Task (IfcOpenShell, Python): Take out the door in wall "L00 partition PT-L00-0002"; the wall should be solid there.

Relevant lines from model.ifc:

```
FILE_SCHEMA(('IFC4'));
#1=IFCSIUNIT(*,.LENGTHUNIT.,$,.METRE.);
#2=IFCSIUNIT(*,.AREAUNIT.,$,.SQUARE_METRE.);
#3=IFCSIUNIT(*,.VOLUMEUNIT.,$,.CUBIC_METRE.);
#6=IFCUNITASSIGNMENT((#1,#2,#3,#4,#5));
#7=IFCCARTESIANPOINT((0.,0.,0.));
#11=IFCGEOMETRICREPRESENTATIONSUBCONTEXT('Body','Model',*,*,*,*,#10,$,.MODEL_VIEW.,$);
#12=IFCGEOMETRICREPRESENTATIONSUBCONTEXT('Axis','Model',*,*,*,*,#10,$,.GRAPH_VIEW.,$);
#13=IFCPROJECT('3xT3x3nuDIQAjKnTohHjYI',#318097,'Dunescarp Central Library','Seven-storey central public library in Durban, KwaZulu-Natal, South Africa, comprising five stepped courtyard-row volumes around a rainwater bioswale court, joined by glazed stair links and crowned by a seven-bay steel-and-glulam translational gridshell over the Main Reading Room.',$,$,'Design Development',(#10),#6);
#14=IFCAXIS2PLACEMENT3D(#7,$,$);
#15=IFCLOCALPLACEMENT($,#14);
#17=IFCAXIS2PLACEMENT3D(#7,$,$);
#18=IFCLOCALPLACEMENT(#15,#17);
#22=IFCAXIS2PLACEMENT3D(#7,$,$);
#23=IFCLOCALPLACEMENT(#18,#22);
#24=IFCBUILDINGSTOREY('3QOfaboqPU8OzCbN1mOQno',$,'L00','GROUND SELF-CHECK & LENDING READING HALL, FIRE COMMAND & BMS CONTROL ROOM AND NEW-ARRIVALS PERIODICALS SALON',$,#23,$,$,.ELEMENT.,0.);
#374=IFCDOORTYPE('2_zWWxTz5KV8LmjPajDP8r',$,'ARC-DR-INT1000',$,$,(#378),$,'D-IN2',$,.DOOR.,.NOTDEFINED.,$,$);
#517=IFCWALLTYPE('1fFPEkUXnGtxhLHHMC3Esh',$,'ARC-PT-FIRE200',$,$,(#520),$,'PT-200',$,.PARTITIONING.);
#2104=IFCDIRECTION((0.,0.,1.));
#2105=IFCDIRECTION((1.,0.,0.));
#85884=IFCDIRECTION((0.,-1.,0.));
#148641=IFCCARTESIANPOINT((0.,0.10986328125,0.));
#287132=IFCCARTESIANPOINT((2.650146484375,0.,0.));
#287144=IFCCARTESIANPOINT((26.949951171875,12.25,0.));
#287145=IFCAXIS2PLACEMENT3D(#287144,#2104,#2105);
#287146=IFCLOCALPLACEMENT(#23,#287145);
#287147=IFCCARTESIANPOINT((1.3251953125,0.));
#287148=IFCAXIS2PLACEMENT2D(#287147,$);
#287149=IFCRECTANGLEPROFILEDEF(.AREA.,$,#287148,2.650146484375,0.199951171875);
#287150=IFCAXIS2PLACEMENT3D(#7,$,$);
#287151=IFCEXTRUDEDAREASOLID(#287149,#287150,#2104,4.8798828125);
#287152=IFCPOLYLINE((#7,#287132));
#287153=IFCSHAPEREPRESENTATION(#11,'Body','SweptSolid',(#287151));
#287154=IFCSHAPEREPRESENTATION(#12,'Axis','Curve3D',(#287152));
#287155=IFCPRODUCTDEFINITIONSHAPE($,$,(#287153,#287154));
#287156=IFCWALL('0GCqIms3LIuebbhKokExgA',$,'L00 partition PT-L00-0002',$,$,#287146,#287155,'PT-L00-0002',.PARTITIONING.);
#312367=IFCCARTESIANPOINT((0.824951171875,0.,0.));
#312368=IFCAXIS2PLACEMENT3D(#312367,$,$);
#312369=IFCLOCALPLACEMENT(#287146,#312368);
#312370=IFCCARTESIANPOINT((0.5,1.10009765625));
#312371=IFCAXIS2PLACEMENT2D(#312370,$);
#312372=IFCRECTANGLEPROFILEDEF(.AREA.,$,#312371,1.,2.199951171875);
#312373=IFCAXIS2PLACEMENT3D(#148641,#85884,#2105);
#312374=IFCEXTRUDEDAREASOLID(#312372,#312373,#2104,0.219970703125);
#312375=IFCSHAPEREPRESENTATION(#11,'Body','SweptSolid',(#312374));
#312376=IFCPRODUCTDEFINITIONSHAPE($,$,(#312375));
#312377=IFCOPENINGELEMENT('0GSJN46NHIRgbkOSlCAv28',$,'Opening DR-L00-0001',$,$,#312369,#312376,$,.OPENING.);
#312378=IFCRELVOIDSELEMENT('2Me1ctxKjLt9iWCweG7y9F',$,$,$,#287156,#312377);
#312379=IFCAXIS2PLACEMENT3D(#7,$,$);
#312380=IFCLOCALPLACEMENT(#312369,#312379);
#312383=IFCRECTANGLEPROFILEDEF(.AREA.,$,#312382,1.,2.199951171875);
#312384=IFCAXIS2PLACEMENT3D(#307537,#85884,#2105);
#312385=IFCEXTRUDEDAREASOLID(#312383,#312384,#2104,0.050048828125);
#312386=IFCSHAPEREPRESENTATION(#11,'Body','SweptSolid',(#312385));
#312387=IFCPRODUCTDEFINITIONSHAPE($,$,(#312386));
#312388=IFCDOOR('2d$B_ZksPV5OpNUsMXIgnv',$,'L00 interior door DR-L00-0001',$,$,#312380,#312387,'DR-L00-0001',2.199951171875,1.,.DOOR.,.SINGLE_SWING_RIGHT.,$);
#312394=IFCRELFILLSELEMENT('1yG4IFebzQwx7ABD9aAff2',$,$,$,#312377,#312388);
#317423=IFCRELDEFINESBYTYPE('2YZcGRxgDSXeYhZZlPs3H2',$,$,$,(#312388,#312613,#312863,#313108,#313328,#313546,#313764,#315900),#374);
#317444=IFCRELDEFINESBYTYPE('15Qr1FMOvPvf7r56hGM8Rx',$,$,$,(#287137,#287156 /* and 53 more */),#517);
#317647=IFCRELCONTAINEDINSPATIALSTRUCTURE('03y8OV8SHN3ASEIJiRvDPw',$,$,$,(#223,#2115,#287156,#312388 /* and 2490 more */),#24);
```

```python
import ifcopenshell
import ifcopenshell.api.feature
import ifcopenshell.api.root
import ifcopenshell.geom
import ifcopenshell.util.shape

model = ifcopenshell.open("model.ifc")
settings = ifcopenshell.geom.settings()


def volume(element):
    """Net volume in cubic metres, openings subtracted."""
    shape = ifcopenshell.geom.create_shape(settings, element)
    return ifcopenshell.util.shape.get_volume(shape.geometry)


door = model.by_guid("2d$B_ZksPV5OpNUsMXIgnv")
opening = door.FillsVoids[0].RelatingOpeningElement
wall = opening.VoidsElements[0].RelatingBuildingElement
before = volume(wall)

ifcopenshell.api.root.remove_product(model, product=door)
ifcopenshell.api.feature.remove_feature(model, feature=opening)

after = volume(wall)

print(f"wall volume {before:.3f} -> {after:.3f} m3")

model.write("model-out.ifc")
```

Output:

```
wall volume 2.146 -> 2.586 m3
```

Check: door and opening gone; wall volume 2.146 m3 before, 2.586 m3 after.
